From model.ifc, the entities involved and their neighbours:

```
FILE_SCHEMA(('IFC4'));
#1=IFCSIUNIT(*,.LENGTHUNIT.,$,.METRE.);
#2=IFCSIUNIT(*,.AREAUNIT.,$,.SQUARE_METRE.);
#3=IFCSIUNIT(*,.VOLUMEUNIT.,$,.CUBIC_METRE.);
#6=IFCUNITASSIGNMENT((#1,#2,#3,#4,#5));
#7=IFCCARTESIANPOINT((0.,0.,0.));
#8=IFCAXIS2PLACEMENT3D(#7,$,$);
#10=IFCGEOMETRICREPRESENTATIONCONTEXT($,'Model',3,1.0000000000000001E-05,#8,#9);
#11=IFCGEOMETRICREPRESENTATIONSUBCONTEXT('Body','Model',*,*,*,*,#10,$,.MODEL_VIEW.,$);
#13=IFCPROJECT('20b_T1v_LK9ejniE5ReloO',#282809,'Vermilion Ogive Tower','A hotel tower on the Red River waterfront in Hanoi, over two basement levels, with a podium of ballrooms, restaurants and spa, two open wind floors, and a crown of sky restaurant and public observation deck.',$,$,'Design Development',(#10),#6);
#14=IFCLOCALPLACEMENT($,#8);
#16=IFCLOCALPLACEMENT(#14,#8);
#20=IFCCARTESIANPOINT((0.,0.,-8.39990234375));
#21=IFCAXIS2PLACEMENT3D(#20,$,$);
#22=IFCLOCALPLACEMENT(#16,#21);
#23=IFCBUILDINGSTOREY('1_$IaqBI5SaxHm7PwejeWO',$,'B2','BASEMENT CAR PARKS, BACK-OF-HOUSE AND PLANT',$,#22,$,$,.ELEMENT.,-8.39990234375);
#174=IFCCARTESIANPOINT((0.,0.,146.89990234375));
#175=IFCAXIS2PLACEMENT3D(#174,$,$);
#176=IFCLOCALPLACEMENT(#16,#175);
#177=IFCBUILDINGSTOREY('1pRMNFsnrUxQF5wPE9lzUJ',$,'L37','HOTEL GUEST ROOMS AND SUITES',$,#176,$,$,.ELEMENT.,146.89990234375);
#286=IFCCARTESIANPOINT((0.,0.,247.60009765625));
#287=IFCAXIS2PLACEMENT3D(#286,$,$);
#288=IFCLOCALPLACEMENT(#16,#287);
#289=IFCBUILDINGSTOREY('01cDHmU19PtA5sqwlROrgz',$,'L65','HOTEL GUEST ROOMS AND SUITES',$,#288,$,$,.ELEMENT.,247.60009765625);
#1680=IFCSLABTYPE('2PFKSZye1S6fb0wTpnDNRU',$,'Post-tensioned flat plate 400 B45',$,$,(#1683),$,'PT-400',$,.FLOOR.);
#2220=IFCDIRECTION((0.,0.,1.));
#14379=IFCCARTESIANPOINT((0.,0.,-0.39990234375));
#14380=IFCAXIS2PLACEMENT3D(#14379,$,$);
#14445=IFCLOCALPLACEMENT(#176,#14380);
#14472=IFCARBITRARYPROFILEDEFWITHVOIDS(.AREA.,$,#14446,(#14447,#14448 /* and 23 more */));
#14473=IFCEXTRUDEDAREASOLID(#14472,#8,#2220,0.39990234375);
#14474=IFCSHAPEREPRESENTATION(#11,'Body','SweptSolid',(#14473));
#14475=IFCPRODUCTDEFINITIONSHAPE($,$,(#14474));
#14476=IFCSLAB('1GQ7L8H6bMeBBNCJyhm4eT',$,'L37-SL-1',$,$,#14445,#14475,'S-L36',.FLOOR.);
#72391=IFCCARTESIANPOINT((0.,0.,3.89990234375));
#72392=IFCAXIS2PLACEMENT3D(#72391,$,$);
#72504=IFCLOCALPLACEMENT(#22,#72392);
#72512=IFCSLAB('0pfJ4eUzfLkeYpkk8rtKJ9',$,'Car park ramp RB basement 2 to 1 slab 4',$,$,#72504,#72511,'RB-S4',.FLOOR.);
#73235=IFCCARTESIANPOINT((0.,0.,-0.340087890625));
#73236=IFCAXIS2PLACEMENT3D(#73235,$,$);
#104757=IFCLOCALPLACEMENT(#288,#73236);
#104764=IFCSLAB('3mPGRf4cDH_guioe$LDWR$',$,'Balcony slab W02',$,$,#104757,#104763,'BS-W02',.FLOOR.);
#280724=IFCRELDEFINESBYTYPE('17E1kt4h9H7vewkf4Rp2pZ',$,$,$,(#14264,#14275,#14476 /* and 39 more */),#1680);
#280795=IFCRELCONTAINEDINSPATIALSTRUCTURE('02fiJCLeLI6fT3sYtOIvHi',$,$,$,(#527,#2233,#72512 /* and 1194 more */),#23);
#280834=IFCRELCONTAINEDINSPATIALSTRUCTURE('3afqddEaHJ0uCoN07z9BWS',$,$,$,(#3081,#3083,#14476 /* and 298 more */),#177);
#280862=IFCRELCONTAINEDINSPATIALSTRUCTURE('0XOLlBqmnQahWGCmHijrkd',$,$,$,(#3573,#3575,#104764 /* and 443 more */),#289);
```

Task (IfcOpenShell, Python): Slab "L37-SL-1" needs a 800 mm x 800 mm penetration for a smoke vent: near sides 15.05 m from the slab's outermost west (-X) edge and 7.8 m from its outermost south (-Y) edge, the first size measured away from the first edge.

```python
import numpy as np
import ifcopenshell
import ifcopenshell.api.feature
import ifcopenshell.api.geometry
import ifcopenshell.api.root
import ifcopenshell.geom
import ifcopenshell.util.placement
import ifcopenshell.util.representation
import ifcopenshell.util.shape
import ifcopenshell.util.unit

model = ifcopenshell.open("model.ifc")
unit_scale = ifcopenshell.util.unit.calculate_unit_scale(model)
settings = ifcopenshell.geom.settings()


def volume(element):
    """Net volume in cubic metres, openings subtracted."""
    shape = ifcopenshell.geom.create_shape(settings, element)
    return ifcopenshell.util.shape.get_volume(shape.geometry)


slab = model.by_id(14476)
before = volume(slab)

# Extent in the slab's own axes, in metres. The edges named are its -X and -Y sides.
slab_shape = ifcopenshell.geom.create_shape(settings, slab)
vertices = ifcopenshell.util.shape.get_vertices(slab_shape.geometry)
x_min, y_min, bottom = vertices.min(axis=0)
top = vertices[:, 2].max()

opening = ifcopenshell.api.root.create_entity(model, ifc_class="IfcOpeningElement", name="Smoke vent opening", predefined_type="OPENING")
context = ifcopenshell.util.representation.get_context(model, "Model", "Body", "MODEL_VIEW")
width, depth = 0.8, 0.8
outline = [(0.0, 0.0), (width, 0.0), (width, depth), (0.0, depth), (0.0, 0.0)]
# Overshoot both faces by 50 mm so the cut is clean.
shape = ifcopenshell.api.geometry.add_slab_representation(
    model, context=context, depth=top - bottom + 0.1, polyline=outline
)
ifcopenshell.api.geometry.assign_representation(model, product=opening, representation=shape)

matrix = ifcopenshell.util.placement.get_local_placement(slab.ObjectPlacement)
matrix[:, 3] = matrix @ np.append(np.array([x_min + 15.05, y_min + 7.8, bottom - 0.05]) / unit_scale, 1.0)
ifcopenshell.api.geometry.edit_object_placement(model, product=opening, matrix=matrix, is_si=False)
ifcopenshell.api.feature.add_feature(model, feature=opening, element=slab)

after = volume(slab)

print(f"slab volume {before:.3f} -> {after:.3f} m3")

model.write("model_v2.ifc")
```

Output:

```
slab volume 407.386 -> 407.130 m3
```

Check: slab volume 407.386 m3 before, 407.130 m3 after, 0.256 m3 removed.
